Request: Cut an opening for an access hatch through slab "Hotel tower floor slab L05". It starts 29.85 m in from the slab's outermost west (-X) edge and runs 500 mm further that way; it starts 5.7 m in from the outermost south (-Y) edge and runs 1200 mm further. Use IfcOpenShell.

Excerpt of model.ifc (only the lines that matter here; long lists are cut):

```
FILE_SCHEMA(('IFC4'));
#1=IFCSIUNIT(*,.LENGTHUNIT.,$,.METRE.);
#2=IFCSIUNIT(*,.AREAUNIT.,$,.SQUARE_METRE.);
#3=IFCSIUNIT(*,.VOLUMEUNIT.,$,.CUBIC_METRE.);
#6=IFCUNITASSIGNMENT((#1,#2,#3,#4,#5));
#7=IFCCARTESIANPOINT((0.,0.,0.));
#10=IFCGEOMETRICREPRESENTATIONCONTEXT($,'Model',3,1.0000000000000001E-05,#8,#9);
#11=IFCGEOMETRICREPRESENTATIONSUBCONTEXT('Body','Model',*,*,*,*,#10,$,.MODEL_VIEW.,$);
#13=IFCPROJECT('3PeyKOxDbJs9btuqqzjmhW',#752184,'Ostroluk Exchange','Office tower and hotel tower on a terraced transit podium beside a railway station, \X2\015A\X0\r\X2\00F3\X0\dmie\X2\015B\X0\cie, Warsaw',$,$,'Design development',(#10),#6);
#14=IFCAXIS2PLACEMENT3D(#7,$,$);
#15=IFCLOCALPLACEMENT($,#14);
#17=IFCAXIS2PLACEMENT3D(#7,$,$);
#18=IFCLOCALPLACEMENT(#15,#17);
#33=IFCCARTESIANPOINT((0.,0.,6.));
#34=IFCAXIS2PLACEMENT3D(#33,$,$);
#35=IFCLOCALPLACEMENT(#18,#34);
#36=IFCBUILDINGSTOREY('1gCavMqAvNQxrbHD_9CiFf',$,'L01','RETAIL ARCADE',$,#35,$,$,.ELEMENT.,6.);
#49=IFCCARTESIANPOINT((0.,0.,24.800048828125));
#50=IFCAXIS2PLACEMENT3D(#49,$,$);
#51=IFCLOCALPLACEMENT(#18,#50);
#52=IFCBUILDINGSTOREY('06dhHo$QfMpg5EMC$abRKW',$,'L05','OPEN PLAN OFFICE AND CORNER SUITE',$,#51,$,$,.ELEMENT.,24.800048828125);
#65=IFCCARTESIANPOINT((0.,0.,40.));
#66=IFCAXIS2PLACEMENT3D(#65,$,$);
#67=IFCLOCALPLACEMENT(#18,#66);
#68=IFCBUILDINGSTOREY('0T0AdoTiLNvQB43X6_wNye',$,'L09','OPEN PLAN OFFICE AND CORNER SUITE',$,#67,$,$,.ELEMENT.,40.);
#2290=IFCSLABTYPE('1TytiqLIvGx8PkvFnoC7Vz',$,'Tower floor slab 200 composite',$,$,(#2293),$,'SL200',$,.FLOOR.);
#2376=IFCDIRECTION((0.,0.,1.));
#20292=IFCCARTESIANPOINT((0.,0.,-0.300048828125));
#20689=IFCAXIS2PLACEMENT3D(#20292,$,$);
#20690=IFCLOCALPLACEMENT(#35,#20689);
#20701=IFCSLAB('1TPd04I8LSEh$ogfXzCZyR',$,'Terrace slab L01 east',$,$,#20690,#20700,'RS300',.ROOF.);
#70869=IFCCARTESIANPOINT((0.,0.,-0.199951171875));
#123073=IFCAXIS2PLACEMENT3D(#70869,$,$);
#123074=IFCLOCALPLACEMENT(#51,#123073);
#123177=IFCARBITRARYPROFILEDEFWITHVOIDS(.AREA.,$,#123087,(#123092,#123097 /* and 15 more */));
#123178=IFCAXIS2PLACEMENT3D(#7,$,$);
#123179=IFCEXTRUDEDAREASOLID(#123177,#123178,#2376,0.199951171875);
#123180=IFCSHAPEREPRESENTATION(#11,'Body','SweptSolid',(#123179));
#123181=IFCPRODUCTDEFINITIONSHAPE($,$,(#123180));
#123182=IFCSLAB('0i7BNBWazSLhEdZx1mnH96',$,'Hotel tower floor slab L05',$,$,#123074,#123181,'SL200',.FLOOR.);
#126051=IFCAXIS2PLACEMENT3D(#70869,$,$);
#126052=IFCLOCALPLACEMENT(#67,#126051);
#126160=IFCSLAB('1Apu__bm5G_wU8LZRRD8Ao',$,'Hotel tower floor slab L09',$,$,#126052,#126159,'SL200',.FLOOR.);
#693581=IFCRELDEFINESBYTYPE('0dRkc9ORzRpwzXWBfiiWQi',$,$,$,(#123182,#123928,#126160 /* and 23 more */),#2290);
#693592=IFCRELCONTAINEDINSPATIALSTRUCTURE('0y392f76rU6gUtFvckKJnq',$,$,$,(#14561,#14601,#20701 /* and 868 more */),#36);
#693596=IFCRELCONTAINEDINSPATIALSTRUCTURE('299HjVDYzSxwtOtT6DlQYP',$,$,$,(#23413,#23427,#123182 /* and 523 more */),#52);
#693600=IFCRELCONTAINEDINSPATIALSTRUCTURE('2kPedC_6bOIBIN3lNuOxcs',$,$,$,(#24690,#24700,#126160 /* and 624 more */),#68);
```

```python
import numpy as np
import ifcopenshell
import ifcopenshell.api.feature
import ifcopenshell.api.geometry
import ifcopenshell.api.root
import ifcopenshell.geom
import ifcopenshell.util.placement
import ifcopenshell.util.representation
import ifcopenshell.util.shape
import ifcopenshell.util.unit

model = ifcopenshell.open("model.ifc")
unit_scale = ifcopenshell.util.unit.calculate_unit_scale(model)
settings = ifcopenshell.geom.settings()


def volume(element):
    """Net volume in cubic metres, openings subtracted."""
    shape = ifcopenshell.geom.create_shape(settings, element)
    return ifcopenshell.util.shape.get_volume(shape.geometry)


slab = model.by_guid("0i7BNBWazSLhEdZx1mnH96")
before = volume(slab)

# Extent in the slab's own axes, in metres. The edges named are its -X and -Y sides.
slab_shape = ifcopenshell.geom.create_shape(settings, slab)
vertices = ifcopenshell.util.shape.get_vertices(slab_shape.geometry)
x_min, y_min, bottom = vertices.min(axis=0)
top = vertices[:, 2].max()

opening = ifcopenshell.api.root.create_entity(model, ifc_class="IfcOpeningElement", name="Access hatch opening", predefined_type="OPENING")
context = ifcopenshell.util.representation.get_context(model, "Model", "Body", "MODEL_VIEW")
width, depth = 0.5, 1.2
outline = [(0.0, 0.0), (width, 0.0), (width, depth), (0.0, depth), (0.0, 0.0)]
# Overshoot both faces by 50 mm so the cut is clean.
shape = ifcopenshell.api.geometry.add_slab_representation(
    model, context=context, depth=top - bottom + 0.1, polyline=outline
)
ifcopenshell.api.geometry.assign_representation(model, product=opening, representation=shape)

matrix = ifcopenshell.util.placement.get_local_placement(slab.ObjectPlacement)
matrix[:, 3] = matrix @ np.append(np.array([x_min + 29.85, y_min + 5.7, bottom - 0.05]) / unit_scale, 1.0)
ifcopenshell.api.geometry.edit_object_placement(model, product=opening, matrix=matrix, is_si=False)
ifcopenshell.api.feature.add_feature(model, feature=opening, element=slab)

after = volume(slab)

print(f"slab volume {before:.3f} -> {after:.3f} m3")

model.write("model-out.ifc")
```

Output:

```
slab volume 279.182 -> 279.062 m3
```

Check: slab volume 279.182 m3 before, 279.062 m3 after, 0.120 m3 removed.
